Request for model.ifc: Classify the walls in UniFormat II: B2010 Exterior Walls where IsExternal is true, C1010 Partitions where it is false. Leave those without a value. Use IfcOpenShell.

First a look at what the model holds.

```python
import ifcopenshell
import ifcopenshell.util.element

model = ifcopenshell.open("model.ifc")
print(model.schema)
print("classifications:", [c.Name for c in model.by_type("IfcClassification")])
values = [ifcopenshell.util.element.get_pset(e, "Pset_WallCommon", "IsExternal") for e in model.by_type("IfcWall")]
for value in (True, False, None):
    print("IsExternal", value, values.count(value))
```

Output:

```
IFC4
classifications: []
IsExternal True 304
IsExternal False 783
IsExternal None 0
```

```python
import ifcopenshell
import ifcopenshell.api.classification
import ifcopenshell.util.element

model = ifcopenshell.open("model.ifc")

system = ifcopenshell.api.classification.add_classification(model, classification="UniFormat II")

walls = model.by_type("IfcWall")
external = {e: ifcopenshell.util.element.get_pset(e, "Pset_WallCommon", "IsExternal") for e in walls}
for flag, code, name in ((True, "B2010", "Exterior Walls"), (False, "C1010", "Partitions")):
    products = [e for e in walls if external[e] is flag]
    ifcopenshell.api.classification.add_reference(
        model, products=products, classification=system, identification=code, name=name
    )
    print(code, len(products))

model.write("model_edited.ifc")
```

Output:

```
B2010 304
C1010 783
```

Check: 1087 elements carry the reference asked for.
